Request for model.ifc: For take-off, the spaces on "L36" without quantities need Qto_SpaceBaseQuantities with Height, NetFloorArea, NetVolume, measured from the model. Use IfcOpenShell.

First a look at what the model holds.

```python
import ifcopenshell
import ifcopenshell.util.element
import ifcopenshell.util.unit

model = ifcopenshell.open("model.ifc")
print(model.schema)
for unit_type in ("LENGTHUNIT", "AREAUNIT", "VOLUMEUNIT"):
    print(unit_type, ifcopenshell.util.unit.calculate_unit_scale(model, unit_type))
storey = next(s for s in model.by_type("IfcBuildingStorey") if s.Name == "L36")
spaces = [e for e in ifcopenshell.util.element.get_decomposition(storey) if e.is_a("IfcSpace")]
for e in sorted(spaces, key=lambda e: e.id()):
    print(e.id(), e.is_a(), e.Name, list(ifcopenshell.util.element.get_psets(e, qtos_only=True)), sep=" | ")
```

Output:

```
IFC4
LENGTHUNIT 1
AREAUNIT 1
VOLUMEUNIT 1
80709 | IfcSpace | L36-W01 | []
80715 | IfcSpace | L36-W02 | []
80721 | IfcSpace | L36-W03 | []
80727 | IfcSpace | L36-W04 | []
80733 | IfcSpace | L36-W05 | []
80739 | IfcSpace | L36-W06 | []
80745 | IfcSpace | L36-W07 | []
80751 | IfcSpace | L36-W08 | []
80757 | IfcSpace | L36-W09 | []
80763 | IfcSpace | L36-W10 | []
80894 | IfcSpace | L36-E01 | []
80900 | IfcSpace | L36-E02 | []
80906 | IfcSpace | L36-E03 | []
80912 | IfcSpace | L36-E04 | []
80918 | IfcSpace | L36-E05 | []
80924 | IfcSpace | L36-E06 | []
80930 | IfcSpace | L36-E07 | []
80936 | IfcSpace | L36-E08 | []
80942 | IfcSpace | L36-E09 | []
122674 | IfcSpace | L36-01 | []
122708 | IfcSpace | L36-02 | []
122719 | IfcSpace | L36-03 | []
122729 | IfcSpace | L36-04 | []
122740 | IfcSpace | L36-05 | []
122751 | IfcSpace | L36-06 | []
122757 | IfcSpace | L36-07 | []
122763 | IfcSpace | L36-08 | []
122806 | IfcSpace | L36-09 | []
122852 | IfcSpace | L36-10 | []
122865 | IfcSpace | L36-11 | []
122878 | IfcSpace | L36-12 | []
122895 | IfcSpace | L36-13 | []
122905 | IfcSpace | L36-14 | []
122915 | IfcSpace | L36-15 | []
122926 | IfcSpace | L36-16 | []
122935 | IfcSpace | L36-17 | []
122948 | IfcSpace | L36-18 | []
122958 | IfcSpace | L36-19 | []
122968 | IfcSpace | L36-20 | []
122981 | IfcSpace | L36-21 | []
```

```python
import ifcopenshell
import ifcopenshell.api.pset
import ifcopenshell.geom
import ifcopenshell.util.element
import ifcopenshell.util.shape
import ifcopenshell.util.unit

model = ifcopenshell.open("model.ifc")
unit_scale = ifcopenshell.util.unit.calculate_unit_scale(model)
area_scale = ifcopenshell.util.unit.calculate_unit_scale(model, "AREAUNIT")
volume_scale = ifcopenshell.util.unit.calculate_unit_scale(model, "VOLUMEUNIT")
settings = ifcopenshell.geom.settings()

storey = next(s for s in model.by_type("IfcBuildingStorey") if s.Name == "L36")
spaces = [e for e in ifcopenshell.util.element.get_decomposition(storey) if e.is_a("IfcSpace")]

for e in sorted(spaces, key=lambda e: e.id()):
    if ifcopenshell.util.element.get_psets(e, qtos_only=True, should_inherit=False):
        continue
    # Geometry comes back in metres, in the element's own axes.
    shape = ifcopenshell.geom.create_shape(settings, e)
    values = {
        "Height": ifcopenshell.util.shape.get_z(shape.geometry) / unit_scale,
        "NetFloorArea": ifcopenshell.util.shape.get_footprint_area(shape.geometry) / area_scale,
        "NetVolume": ifcopenshell.util.shape.get_volume(shape.geometry) / volume_scale,
    }
    qto = ifcopenshell.api.pset.add_qto(model, product=e, name="Qto_SpaceBaseQuantities")
    ifcopenshell.api.pset.edit_qto(model, qto=qto, properties=values)
    print(e.id(), {k: round(v, 3) for k, v in values.items()})

model.write("model_rev.ifc")
```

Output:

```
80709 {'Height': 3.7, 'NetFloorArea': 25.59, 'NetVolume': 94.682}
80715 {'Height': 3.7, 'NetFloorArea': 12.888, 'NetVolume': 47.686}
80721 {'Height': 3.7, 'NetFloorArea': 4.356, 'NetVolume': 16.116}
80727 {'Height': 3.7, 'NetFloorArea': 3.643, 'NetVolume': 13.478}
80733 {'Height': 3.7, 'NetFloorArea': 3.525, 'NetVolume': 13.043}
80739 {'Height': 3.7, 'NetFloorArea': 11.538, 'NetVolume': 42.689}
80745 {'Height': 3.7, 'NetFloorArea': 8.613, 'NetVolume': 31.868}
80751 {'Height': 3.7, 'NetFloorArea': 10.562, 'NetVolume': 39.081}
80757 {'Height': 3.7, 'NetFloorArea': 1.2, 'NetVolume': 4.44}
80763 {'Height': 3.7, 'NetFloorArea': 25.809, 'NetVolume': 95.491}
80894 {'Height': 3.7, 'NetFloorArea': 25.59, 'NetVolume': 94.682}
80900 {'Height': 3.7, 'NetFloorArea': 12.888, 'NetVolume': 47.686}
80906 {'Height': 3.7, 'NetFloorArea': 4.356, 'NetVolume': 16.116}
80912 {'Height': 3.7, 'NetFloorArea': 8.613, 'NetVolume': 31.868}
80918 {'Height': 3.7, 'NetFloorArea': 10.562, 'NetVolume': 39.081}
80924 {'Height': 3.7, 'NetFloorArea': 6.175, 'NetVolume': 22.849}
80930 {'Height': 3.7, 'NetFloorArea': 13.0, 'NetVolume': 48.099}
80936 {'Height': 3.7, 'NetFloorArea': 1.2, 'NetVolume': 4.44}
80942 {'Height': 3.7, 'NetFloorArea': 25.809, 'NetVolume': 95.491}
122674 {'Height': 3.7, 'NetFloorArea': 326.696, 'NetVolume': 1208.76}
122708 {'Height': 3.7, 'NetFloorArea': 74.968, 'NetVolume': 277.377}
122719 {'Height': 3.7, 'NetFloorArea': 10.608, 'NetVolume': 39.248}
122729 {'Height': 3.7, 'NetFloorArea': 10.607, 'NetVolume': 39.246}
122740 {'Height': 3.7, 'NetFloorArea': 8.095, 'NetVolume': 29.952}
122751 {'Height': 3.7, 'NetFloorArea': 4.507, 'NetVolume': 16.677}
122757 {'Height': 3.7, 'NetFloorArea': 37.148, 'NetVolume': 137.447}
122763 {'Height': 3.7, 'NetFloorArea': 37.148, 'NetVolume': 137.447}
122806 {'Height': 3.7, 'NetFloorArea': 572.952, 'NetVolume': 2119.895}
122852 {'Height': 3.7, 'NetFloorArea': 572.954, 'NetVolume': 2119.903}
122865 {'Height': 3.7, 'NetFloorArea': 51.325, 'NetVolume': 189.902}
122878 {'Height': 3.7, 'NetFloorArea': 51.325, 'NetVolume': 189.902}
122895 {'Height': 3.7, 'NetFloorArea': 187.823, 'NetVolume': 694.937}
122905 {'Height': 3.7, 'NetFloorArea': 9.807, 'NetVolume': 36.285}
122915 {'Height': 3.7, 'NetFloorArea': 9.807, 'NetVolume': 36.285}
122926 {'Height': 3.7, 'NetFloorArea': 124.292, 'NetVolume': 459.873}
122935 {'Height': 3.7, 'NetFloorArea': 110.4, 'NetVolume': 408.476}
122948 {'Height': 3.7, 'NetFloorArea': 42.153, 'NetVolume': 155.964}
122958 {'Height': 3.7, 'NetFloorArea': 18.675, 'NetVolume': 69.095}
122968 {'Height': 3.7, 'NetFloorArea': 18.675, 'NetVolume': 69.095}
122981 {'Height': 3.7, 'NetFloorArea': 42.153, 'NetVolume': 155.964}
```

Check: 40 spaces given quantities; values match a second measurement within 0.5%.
